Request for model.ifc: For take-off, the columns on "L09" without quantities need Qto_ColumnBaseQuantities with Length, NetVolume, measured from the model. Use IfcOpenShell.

First a look at what the model holds.

```python
import ifcopenshell
import ifcopenshell.util.element
import ifcopenshell.util.unit

model = ifcopenshell.open("model.ifc")
print(model.schema)
for unit_type in ("LENGTHUNIT", "AREAUNIT", "VOLUMEUNIT"):
    print(unit_type, ifcopenshell.util.unit.calculate_unit_scale(model, unit_type))
storey = next(s for s in model.by_type("IfcBuildingStorey") if s.Name == "L09")
columns = [e for e in ifcopenshell.util.element.get_decomposition(storey) if e.is_a("IfcColumn")]
for e in sorted(columns, key=lambda e: e.id()):
    print(e.id(), e.is_a(), e.Name, list(ifcopenshell.util.element.get_psets(e, qtos_only=True)), sep=" | ")
```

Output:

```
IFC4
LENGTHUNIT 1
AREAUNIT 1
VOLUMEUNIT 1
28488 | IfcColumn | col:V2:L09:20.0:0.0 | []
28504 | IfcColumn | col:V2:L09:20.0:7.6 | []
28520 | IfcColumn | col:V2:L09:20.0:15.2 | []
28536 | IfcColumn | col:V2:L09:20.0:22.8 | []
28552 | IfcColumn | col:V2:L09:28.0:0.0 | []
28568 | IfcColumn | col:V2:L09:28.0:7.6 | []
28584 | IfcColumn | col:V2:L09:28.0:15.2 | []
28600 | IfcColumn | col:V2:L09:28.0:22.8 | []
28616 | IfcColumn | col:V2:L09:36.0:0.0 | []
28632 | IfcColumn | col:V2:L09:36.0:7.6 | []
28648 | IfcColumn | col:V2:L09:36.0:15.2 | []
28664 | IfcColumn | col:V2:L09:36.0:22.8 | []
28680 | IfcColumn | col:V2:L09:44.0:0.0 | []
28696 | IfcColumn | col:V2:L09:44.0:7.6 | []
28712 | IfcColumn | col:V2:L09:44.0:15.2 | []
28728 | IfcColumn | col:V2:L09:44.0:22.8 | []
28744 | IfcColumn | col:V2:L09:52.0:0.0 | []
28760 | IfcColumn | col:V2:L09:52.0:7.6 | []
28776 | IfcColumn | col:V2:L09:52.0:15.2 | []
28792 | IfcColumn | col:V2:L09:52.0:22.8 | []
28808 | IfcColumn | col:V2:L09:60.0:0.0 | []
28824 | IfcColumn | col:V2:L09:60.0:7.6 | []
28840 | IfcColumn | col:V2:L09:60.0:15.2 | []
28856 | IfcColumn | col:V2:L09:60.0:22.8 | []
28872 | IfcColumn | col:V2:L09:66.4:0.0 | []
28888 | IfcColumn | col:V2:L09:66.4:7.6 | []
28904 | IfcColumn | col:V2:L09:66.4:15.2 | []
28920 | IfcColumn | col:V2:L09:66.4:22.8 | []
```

```python
import ifcopenshell
import ifcopenshell.api.pset
import ifcopenshell.geom
import ifcopenshell.util.element
import ifcopenshell.util.shape
import ifcopenshell.util.unit

model = ifcopenshell.open("model.ifc")
unit_scale = ifcopenshell.util.unit.calculate_unit_scale(model)
volume_scale = ifcopenshell.util.unit.calculate_unit_scale(model, "VOLUMEUNIT")
settings = ifcopenshell.geom.settings()

storey = next(s for s in model.by_type("IfcBuildingStorey") if s.Name == "L09")
columns = [e for e in ifcopenshell.util.element.get_decomposition(storey) if e.is_a("IfcColumn")]

for e in sorted(columns, key=lambda e: e.id()):
    if ifcopenshell.util.element.get_psets(e, qtos_only=True, should_inherit=False):
        continue
    # Geometry comes back in metres, in the element's own axes.
    shape = ifcopenshell.geom.create_shape(settings, e)
    values = {
        "Length": ifcopenshell.util.shape.get_z(shape.geometry) / unit_scale,
        "NetVolume": ifcopenshell.util.shape.get_volume(shape.geometry) / volume_scale,
    }
    qto = ifcopenshell.api.pset.add_qto(model, product=e, name="Qto_ColumnBaseQuantities")
    ifcopenshell.api.pset.edit_qto(model, qto=qto, properties=values)
    print(e.id(), {k: round(v, 3) for k, v in values.items()})

model.write("model_rev.ifc")
```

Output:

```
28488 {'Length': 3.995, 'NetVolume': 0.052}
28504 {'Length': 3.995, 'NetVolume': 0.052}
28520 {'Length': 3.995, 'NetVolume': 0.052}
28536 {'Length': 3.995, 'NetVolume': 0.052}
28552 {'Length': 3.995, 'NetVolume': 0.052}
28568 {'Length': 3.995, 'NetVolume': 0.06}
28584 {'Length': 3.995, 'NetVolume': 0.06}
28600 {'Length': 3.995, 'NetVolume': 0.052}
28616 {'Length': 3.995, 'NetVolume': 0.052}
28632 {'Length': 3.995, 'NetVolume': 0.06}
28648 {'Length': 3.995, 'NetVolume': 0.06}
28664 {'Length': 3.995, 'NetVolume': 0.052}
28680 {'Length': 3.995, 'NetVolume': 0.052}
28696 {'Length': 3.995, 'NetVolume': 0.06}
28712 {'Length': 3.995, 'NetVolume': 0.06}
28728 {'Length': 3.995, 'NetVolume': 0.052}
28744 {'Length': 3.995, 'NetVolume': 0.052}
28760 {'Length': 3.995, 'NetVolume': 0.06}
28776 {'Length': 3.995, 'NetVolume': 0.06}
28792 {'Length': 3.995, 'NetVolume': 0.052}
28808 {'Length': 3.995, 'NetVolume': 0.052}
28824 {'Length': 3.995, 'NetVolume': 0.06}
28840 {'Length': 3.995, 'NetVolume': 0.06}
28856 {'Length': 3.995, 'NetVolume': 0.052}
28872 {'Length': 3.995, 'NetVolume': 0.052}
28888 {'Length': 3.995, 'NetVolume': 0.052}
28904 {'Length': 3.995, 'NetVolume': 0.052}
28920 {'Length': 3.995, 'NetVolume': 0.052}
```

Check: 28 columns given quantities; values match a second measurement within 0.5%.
